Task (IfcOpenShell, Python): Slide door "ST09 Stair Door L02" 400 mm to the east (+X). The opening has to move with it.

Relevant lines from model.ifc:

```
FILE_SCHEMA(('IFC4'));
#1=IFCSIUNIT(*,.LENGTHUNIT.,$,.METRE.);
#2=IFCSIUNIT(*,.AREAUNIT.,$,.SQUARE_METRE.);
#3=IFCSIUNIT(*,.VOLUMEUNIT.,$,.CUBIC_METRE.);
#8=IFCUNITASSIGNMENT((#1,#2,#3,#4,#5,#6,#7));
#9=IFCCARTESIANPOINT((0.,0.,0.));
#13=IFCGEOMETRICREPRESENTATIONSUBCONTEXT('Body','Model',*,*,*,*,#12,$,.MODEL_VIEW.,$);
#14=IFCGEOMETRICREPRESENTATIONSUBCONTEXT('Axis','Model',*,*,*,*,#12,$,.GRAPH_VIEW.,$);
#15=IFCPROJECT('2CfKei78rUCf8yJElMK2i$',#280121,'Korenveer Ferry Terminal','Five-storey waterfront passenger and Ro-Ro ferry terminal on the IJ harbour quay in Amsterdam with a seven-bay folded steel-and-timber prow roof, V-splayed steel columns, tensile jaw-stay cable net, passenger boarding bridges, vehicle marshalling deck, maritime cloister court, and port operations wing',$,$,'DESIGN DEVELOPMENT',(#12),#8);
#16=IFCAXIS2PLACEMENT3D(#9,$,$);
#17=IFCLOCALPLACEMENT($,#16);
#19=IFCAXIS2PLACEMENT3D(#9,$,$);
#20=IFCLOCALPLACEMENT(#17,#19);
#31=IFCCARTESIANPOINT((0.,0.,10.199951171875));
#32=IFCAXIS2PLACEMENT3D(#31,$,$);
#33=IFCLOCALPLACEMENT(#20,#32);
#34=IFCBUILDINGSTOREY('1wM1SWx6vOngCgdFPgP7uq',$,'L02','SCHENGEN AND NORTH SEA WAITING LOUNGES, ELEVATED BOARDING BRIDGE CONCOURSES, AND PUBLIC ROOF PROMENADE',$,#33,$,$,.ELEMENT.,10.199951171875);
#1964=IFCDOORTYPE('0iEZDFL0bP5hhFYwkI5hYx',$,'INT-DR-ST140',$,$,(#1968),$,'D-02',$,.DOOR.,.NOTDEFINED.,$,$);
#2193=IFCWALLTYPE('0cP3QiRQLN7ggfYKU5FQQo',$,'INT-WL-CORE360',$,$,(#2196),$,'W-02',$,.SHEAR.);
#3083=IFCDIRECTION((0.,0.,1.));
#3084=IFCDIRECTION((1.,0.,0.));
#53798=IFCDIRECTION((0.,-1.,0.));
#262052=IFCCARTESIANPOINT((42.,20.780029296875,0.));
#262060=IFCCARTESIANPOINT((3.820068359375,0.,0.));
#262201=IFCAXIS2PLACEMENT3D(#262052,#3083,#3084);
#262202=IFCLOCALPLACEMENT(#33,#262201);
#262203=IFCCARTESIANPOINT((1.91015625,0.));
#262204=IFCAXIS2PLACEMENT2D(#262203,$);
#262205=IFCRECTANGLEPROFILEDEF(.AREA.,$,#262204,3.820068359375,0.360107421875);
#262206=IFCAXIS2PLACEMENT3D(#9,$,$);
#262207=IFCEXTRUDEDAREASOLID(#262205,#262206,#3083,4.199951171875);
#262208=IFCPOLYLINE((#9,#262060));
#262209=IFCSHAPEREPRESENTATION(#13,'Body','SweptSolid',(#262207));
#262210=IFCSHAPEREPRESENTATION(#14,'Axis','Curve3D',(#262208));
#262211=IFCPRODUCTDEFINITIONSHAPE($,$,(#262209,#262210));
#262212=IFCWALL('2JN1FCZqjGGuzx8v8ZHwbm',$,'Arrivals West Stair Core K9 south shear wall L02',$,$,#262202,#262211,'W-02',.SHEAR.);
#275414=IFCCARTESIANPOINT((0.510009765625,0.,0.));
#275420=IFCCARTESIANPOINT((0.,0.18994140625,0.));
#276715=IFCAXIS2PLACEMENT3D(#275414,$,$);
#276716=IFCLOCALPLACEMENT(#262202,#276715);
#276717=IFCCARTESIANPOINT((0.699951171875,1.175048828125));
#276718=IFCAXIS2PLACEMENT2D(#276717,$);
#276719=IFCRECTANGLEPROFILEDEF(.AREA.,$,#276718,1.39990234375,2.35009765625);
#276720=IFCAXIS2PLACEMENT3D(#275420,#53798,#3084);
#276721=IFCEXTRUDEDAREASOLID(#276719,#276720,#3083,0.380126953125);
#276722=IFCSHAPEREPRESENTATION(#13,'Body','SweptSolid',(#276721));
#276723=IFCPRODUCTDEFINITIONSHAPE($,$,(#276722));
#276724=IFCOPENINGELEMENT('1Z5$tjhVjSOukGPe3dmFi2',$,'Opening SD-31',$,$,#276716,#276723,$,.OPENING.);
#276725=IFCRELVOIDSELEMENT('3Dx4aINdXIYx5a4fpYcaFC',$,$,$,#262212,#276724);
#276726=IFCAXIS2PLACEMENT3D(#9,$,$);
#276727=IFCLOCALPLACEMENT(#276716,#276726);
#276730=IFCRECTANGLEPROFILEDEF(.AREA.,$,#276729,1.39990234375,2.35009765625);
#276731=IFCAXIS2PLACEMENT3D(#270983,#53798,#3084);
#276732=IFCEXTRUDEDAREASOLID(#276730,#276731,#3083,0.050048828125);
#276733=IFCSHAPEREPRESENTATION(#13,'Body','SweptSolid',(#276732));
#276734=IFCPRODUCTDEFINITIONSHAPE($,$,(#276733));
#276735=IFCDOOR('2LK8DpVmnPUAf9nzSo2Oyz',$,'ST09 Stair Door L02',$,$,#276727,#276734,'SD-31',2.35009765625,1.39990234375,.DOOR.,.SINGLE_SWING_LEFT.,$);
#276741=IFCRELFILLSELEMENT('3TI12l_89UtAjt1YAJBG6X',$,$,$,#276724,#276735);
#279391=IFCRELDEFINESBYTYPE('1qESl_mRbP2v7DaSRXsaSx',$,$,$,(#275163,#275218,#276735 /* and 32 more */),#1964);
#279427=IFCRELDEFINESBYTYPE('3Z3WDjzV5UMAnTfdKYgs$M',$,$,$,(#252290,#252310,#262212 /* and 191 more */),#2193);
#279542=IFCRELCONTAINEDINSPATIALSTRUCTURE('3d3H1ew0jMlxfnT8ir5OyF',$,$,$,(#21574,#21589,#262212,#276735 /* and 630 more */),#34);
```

```python
import ifcopenshell
import ifcopenshell.api.geometry
import ifcopenshell.util.placement

model = ifcopenshell.open("model.ifc")

door = model.by_guid("2LK8DpVmnPUAf9nzSo2Oyz")
opening = door.FillsVoids[0].RelatingOpeningElement
wall = opening.VoidsElements[0].RelatingBuildingElement

wall_matrix = ifcopenshell.util.placement.get_local_placement(wall.ObjectPlacement)
shift = wall_matrix[:3, 0] * 0.4
before = ifcopenshell.util.placement.get_local_placement(door.ObjectPlacement)[:3, 3].copy()

# The door is placed relative to its opening, so it follows when the opening moves.
matrix = ifcopenshell.util.placement.get_local_placement(opening.ObjectPlacement)
matrix[:3, 3] += shift
ifcopenshell.api.geometry.edit_object_placement(
    model, product=opening, matrix=matrix, is_si=False, should_transform_children=True
)

after = ifcopenshell.util.placement.get_local_placement(door.ObjectPlacement)[:3, 3]
print("door moved by", (after - before).round(3) + 0.0)

model.write("model_edited.ifc")
```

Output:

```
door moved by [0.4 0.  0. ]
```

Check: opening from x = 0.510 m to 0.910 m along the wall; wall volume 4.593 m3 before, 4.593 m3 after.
